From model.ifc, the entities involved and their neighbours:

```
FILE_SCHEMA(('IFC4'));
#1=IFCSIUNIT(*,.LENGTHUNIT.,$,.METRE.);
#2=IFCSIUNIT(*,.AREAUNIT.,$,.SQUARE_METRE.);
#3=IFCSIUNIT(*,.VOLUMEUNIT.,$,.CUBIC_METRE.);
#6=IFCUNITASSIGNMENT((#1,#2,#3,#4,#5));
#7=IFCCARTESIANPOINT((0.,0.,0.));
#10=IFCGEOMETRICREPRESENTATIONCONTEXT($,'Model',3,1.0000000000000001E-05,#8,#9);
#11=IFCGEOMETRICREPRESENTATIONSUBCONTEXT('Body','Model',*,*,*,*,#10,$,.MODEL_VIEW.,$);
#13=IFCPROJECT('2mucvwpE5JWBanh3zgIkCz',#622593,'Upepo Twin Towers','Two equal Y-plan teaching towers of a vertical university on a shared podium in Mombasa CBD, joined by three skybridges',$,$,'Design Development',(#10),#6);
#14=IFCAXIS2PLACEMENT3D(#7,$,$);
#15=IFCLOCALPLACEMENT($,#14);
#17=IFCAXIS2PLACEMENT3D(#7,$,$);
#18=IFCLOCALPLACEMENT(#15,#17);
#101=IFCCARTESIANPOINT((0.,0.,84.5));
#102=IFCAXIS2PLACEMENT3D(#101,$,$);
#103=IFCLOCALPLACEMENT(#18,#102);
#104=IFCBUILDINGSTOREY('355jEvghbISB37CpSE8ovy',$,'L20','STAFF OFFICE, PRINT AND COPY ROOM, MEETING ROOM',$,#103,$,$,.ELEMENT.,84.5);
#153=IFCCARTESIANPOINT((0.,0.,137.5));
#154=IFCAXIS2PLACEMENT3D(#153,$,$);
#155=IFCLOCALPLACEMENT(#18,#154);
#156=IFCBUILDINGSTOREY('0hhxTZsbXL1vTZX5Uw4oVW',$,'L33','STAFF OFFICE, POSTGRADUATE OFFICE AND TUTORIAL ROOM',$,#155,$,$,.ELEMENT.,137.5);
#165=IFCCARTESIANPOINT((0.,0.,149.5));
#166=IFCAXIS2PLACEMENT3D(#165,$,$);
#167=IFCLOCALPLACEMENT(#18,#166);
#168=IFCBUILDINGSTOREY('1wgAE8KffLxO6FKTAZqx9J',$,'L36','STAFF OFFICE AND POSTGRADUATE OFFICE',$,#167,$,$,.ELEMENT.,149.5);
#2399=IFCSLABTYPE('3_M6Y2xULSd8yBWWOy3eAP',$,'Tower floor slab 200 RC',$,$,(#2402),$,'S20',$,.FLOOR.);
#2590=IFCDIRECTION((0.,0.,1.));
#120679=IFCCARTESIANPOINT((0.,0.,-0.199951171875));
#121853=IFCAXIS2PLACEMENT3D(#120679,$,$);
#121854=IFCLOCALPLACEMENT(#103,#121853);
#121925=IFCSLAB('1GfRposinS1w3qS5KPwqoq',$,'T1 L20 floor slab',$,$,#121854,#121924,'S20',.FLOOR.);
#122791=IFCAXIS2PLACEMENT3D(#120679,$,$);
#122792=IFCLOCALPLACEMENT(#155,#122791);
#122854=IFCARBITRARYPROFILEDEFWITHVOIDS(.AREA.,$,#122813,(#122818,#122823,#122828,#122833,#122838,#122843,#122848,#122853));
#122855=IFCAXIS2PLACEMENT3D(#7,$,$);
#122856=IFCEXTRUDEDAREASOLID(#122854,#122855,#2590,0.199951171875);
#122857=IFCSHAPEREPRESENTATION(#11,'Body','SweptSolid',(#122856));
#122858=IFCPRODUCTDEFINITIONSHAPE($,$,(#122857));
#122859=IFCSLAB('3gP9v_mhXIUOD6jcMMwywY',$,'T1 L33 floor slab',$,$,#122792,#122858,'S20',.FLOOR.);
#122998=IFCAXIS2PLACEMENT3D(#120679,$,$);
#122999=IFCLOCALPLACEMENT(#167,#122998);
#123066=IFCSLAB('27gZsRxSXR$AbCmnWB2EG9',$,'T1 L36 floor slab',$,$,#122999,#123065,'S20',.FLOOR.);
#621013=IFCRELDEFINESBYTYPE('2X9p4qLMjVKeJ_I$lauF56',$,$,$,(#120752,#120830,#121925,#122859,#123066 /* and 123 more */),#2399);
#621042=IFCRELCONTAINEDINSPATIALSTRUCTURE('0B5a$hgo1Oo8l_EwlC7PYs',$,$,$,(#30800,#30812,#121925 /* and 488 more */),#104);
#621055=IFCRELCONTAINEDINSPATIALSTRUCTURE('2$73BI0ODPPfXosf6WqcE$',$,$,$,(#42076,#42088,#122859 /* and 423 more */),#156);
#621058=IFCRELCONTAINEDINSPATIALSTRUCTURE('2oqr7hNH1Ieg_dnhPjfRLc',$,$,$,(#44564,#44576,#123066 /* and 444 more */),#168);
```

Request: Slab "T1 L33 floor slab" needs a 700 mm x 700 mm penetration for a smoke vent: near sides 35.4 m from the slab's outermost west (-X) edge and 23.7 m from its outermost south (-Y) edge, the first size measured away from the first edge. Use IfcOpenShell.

```python
import numpy as np
import ifcopenshell
import ifcopenshell.api.feature
import ifcopenshell.api.geometry
import ifcopenshell.api.root
import ifcopenshell.geom
import ifcopenshell.util.placement
import ifcopenshell.util.representation
import ifcopenshell.util.shape
import ifcopenshell.util.unit

model = ifcopenshell.open("model.ifc")
unit_scale = ifcopenshell.util.unit.calculate_unit_scale(model)
settings = ifcopenshell.geom.settings()


def volume(element):
    """Net volume in cubic metres, openings subtracted."""
    shape = ifcopenshell.geom.create_shape(settings, element)
    return ifcopenshell.util.shape.get_volume(shape.geometry)


slab = model.by_guid("3gP9v_mhXIUOD6jcMMwywY")
before = volume(slab)

# Extent in the slab's own axes, in metres. The edges named are its -X and -Y sides.
slab_shape = ifcopenshell.geom.create_shape(settings, slab)
vertices = ifcopenshell.util.shape.get_vertices(slab_shape.geometry)
x_min, y_min, bottom = vertices.min(axis=0)
top = vertices[:, 2].max()

opening = ifcopenshell.api.root.create_entity(model, ifc_class="IfcOpeningElement", name="Smoke vent opening", predefined_type="OPENING")
context = ifcopenshell.util.representation.get_context(model, "Model", "Body", "MODEL_VIEW")
width, depth = 0.7, 0.7
outline = [(0.0, 0.0), (width, 0.0), (width, depth), (0.0, depth), (0.0, 0.0)]
# Overshoot both faces by 50 mm so the cut is clean.
shape = ifcopenshell.api.geometry.add_slab_representation(
    model, context=context, depth=top - bottom + 0.1, polyline=outline
)
ifcopenshell.api.geometry.assign_representation(model, product=opening, representation=shape)

matrix = ifcopenshell.util.placement.get_local_placement(slab.ObjectPlacement)
matrix[:, 3] = matrix @ np.append(np.array([x_min + 35.4, y_min + 23.7, bottom - 0.05]) / unit_scale, 1.0)
ifcopenshell.api.geometry.edit_object_placement(model, product=opening, matrix=matrix, is_si=False)
ifcopenshell.api.feature.add_feature(model, feature=opening, element=slab)

after = volume(slab)

print(f"slab volume {before:.3f} -> {after:.3f} m3")

model.write("model_rev.ifc")
```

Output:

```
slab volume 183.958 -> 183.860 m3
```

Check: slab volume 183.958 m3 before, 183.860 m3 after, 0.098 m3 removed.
